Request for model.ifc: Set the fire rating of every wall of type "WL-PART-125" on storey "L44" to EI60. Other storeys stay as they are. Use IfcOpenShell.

First a look at what the model holds.

```python
import ifcopenshell
import ifcopenshell.util.element

model = ifcopenshell.open("model.ifc")
print(model.schema)
storey = next(s for s in model.by_type("IfcBuildingStorey") if s.Name == "L44")
walls = [e for e in ifcopenshell.util.element.get_decomposition(storey) if e.is_a("IfcWall")]
seen = {}
for e in walls:
    element_type = ifcopenshell.util.element.get_type(e)
    key = (element_type.Name if element_type != e and element_type else None, ifcopenshell.util.element.get_pset(e, "Pset_WallCommon", "FireRating"))
    seen[key] = seen.get(key, 0) + 1
for (name, value), count in sorted(seen.items(), key=str):
    print(count, "x", name, "|", value)
```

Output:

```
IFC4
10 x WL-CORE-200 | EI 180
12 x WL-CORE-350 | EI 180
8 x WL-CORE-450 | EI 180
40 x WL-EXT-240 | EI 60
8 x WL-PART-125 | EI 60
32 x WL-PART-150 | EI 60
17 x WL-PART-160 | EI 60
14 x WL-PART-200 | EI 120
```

```python
import ifcopenshell
import ifcopenshell.api.pset
import ifcopenshell.util.element

model = ifcopenshell.open("model.ifc")

storey = next(s for s in model.by_type("IfcBuildingStorey") if s.Name == "L44")
walls = [e for e in ifcopenshell.util.element.get_decomposition(storey) if e.is_a("IfcWall")]

count = 0
for e in walls:
    element_type = ifcopenshell.util.element.get_type(e)
    if element_type in (None, e) or element_type.Name != "WL-PART-125":
        continue
    found = ifcopenshell.util.element.get_pset(e, "Pset_WallCommon", should_inherit=False)
    if found:
        pset = model.by_id(found["id"])
        if len(ifcopenshell.util.element.get_elements_by_pset(pset)) > 1:
            pset = ifcopenshell.api.pset.unshare_pset(model, products=[e], pset=pset)[0]
    else:
        pset = ifcopenshell.api.pset.add_pset(model, product=e, name="Pset_WallCommon")
    ifcopenshell.api.pset.edit_pset(model, pset=pset, properties={"FireRating": "EI60"})
    count += 1

print(count, "walls updated")

model.write("model_edited.ifc")
```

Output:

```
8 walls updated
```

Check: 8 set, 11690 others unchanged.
